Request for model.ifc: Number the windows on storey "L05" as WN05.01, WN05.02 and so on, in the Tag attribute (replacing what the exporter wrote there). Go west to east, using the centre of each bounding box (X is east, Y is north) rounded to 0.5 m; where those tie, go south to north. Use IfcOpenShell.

First a look at what the model holds.

```python
import ifcopenshell
import ifcopenshell.util.element
import ifcopenshell.util.placement

model = ifcopenshell.open("model.ifc")
print(model.schema)
storey = next(s for s in model.by_type("IfcBuildingStorey") if s.Name == "L05")
windows = [e for e in ifcopenshell.util.element.get_decomposition(storey) if e.is_a("IfcWindow")]
for e in sorted(windows, key=lambda e: e.id()):
    origin = ifcopenshell.util.placement.get_local_placement(e.ObjectPlacement)[:3, 3]
    print(e.id(), e.Tag, e.Name, origin.round(2) + 0.0, sep=" | ")
```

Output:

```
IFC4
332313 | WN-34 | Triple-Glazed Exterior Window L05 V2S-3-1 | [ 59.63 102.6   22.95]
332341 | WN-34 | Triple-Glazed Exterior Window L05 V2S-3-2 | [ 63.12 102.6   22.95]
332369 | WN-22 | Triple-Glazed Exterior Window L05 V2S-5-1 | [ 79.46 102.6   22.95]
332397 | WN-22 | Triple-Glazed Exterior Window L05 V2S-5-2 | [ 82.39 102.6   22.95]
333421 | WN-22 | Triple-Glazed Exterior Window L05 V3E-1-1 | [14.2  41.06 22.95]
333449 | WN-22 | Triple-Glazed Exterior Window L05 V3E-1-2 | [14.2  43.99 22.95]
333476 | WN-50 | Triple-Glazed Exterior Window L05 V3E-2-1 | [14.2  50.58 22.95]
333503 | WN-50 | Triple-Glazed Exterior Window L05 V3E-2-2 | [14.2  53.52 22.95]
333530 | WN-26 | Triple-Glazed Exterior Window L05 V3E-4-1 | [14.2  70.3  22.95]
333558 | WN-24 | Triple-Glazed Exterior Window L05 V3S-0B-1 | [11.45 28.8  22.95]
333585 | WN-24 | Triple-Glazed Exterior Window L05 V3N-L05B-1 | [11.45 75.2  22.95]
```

```python
import ifcopenshell
import ifcopenshell.geom
import ifcopenshell.util.element
import ifcopenshell.util.shape

model = ifcopenshell.open("model.ifc")
settings = ifcopenshell.geom.settings()
settings.set("use-world-coords", True)


def centre(element):
    shape = ifcopenshell.geom.create_shape(settings, element)
    return ifcopenshell.util.shape.get_bbox_centroid(shape.geometry)


storey = next(s for s in model.by_type("IfcBuildingStorey") if s.Name == "L05")
windows = [e for e in ifcopenshell.util.element.get_decomposition(storey) if e.is_a("IfcWindow")]

# Insertion points can sit at a corner or the storey origin, so sort by the geometry (in metres).
centres = {e: centre(e) for e in windows}
windows.sort(key=lambda e: (round(centres[e][0] / 0.5), centres[e][1]))

for i, e in enumerate(windows, start=1):
    number = f"WN05.{i:02d}"
    e.Tag = number
    print(e.id(), number)

model.write("model_v2.ifc")
```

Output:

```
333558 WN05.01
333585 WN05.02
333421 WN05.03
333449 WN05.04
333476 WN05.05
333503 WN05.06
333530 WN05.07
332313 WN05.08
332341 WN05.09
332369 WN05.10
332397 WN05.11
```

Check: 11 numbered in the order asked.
